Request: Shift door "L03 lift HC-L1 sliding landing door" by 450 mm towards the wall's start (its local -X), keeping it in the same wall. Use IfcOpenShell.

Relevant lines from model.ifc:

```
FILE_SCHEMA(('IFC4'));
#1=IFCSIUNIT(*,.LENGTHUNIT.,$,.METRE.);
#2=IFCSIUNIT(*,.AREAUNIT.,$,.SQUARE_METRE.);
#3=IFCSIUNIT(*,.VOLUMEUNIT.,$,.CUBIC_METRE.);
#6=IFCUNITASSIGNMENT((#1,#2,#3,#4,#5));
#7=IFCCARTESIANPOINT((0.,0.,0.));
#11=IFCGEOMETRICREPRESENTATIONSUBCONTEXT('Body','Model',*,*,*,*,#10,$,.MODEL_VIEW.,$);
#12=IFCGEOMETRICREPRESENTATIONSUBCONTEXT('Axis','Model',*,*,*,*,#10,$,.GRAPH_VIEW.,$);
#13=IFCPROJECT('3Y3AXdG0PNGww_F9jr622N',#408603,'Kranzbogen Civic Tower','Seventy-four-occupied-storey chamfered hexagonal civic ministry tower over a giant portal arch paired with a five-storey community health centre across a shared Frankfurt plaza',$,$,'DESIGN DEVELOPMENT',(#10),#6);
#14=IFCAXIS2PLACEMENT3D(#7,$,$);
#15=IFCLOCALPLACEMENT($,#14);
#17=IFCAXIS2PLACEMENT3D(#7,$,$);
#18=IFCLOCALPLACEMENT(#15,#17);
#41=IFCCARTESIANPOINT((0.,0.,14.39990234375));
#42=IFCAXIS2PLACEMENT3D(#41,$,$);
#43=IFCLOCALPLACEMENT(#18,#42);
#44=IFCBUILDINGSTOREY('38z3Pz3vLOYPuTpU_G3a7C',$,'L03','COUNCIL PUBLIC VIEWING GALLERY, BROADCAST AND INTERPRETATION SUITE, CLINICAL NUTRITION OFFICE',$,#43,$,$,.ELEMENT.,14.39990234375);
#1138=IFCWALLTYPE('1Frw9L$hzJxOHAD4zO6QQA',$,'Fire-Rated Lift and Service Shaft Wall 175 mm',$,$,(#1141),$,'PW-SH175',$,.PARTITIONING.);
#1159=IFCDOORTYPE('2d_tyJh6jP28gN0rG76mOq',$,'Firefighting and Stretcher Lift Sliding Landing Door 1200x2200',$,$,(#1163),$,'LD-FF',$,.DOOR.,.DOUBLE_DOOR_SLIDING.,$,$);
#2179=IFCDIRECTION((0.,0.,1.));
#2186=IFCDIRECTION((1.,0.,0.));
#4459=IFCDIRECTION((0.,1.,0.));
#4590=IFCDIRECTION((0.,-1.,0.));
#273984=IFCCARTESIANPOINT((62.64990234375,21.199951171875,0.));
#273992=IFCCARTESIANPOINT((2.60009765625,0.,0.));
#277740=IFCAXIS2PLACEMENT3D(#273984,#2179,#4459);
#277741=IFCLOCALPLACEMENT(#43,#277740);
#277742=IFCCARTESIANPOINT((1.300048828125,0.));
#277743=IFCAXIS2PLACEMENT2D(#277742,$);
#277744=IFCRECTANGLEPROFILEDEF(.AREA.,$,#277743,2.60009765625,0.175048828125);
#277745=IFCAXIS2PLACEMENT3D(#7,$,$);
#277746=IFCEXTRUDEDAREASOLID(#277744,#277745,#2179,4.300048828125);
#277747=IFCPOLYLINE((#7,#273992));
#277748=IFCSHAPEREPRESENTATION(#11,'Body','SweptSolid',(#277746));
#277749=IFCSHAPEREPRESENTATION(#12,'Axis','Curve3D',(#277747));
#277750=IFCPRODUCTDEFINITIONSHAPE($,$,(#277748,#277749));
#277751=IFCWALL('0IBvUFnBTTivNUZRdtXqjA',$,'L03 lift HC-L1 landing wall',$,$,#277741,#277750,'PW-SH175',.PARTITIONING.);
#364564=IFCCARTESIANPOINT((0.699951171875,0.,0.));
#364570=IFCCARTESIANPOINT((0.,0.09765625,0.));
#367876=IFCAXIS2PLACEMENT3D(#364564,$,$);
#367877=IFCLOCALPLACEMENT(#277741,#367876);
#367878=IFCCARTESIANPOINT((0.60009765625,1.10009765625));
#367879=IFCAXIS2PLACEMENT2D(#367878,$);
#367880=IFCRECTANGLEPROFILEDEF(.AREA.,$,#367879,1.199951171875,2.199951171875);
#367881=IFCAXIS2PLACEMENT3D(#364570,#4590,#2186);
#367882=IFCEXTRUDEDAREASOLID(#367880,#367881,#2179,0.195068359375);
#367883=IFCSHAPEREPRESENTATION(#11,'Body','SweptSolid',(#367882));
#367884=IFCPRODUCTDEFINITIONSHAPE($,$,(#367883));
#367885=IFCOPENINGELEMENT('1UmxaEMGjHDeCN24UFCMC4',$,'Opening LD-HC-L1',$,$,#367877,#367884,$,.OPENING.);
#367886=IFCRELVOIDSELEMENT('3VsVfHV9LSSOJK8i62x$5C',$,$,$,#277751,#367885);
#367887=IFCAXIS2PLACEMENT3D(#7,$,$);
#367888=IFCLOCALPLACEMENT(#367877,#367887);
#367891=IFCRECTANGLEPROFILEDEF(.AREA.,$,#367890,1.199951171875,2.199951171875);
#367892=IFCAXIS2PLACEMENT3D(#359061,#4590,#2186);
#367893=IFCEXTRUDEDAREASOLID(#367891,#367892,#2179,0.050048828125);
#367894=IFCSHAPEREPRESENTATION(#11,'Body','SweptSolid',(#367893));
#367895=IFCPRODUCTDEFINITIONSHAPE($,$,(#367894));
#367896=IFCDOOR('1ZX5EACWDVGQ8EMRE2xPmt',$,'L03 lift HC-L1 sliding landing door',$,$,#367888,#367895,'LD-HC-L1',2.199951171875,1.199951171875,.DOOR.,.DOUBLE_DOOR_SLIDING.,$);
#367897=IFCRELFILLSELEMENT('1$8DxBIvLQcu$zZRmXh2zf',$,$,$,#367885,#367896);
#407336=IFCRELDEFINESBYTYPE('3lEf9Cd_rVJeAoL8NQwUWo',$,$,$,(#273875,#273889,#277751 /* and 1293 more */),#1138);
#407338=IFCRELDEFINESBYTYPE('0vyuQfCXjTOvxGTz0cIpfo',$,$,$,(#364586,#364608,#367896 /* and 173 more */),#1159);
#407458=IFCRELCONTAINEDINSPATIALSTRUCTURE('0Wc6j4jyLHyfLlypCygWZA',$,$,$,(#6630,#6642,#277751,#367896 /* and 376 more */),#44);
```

```python
import ifcopenshell
import ifcopenshell.api.geometry
import ifcopenshell.util.placement
import ifcopenshell.util.unit

model = ifcopenshell.open("model.ifc")
unit_scale = ifcopenshell.util.unit.calculate_unit_scale(model)

door = model.by_guid("1ZX5EACWDVGQ8EMRE2xPmt")
opening = door.FillsVoids[0].RelatingOpeningElement
wall = opening.VoidsElements[0].RelatingBuildingElement

wall_matrix = ifcopenshell.util.placement.get_local_placement(wall.ObjectPlacement)
shift = wall_matrix[:3, 0] * -0.45 / unit_scale
before = ifcopenshell.util.placement.get_local_placement(door.ObjectPlacement)[:3, 3].copy()

# The door is placed relative to its opening, so it follows when the opening moves.
matrix = ifcopenshell.util.placement.get_local_placement(opening.ObjectPlacement)
matrix[:3, 3] += shift
ifcopenshell.api.geometry.edit_object_placement(
    model, product=opening, matrix=matrix, is_si=False, should_transform_children=True
)

after = ifcopenshell.util.placement.get_local_placement(door.ObjectPlacement)[:3, 3]
print("door moved by", (after - before).round(3) + 0.0)

model.write("model_updated.ifc")
```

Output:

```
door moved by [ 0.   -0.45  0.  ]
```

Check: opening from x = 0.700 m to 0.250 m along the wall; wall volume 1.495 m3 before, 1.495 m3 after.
